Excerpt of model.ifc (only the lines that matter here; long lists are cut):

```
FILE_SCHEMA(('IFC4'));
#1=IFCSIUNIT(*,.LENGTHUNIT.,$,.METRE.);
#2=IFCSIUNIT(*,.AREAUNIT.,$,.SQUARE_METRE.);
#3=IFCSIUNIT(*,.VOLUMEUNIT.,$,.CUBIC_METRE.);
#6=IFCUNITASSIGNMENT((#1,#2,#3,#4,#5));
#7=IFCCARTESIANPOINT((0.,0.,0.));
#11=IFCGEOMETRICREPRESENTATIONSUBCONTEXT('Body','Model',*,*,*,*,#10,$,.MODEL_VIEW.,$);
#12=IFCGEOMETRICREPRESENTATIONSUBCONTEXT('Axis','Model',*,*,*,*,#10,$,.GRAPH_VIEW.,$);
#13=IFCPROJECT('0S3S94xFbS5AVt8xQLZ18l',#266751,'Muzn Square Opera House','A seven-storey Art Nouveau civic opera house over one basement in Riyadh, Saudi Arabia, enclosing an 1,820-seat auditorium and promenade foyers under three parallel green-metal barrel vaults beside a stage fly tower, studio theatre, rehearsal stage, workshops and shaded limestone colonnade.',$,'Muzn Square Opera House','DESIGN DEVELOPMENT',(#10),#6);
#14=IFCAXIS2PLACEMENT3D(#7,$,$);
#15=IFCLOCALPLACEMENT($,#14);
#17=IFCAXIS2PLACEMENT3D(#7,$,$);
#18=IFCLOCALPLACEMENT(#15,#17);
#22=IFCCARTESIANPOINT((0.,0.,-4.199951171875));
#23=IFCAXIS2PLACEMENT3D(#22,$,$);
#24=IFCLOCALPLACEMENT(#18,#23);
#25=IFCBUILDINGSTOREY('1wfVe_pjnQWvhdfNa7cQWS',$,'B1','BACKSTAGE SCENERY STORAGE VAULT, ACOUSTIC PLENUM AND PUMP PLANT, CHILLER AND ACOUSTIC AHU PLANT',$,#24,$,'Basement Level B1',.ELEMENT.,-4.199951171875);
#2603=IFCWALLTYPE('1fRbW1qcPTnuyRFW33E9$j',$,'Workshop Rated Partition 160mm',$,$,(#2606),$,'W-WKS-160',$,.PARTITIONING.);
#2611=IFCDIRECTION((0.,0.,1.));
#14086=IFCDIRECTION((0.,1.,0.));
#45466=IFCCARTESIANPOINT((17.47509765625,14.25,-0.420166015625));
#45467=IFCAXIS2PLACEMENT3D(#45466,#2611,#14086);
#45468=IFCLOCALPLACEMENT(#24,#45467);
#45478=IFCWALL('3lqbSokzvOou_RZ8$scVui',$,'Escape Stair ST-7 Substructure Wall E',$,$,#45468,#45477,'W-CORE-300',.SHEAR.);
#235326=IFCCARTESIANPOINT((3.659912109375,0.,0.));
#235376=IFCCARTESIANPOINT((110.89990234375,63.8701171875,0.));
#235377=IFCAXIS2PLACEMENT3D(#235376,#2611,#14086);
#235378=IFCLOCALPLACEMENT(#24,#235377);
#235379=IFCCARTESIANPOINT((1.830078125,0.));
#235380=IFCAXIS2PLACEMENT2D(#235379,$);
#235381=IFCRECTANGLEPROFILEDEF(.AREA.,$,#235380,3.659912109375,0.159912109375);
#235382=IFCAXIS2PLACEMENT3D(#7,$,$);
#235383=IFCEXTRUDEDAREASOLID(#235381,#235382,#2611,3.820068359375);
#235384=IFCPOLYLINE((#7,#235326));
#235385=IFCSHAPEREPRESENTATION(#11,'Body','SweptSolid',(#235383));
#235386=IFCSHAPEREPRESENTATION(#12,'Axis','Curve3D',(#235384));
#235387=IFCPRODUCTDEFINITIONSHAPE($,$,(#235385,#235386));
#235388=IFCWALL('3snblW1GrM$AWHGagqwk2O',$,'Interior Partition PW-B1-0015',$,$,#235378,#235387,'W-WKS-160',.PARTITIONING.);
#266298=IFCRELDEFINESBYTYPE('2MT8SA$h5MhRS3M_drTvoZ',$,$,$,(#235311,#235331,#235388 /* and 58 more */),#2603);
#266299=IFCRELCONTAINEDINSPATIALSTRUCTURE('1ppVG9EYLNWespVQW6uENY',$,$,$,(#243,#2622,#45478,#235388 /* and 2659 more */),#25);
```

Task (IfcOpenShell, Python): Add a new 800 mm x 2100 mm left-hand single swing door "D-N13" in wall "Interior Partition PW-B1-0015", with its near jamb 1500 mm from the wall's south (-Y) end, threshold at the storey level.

```python
import numpy as np
import ifcopenshell
import ifcopenshell.api.feature
import ifcopenshell.api.geometry
import ifcopenshell.api.root
import ifcopenshell.api.spatial
import ifcopenshell.geom
import ifcopenshell.util.element
import ifcopenshell.util.placement
import ifcopenshell.util.representation
import ifcopenshell.util.shape
import ifcopenshell.util.unit

model = ifcopenshell.open("model.ifc")
unit_scale = ifcopenshell.util.unit.calculate_unit_scale(model)
settings = ifcopenshell.geom.settings()


def volume(element):
    """Net volume in cubic metres, openings subtracted."""
    shape = ifcopenshell.geom.create_shape(settings, element)
    return ifcopenshell.util.shape.get_volume(shape.geometry)


wall = model.by_guid("3snblW1GrM$AWHGagqwk2O")
storey = ifcopenshell.util.element.get_container(wall, ifc_class="IfcBuildingStorey")
context = ifcopenshell.util.representation.get_context(model, "Model", "Body", "MODEL_VIEW")
before = volume(wall)

width, height, from_end, sill = 0.8, 2.1, 1.5, 0.0  # metres

# The wall runs along its own X axis, and the end named is its -X end.
wall_shape = ifcopenshell.geom.create_shape(settings, wall)
x, y, z = ifcopenshell.util.shape.get_vertices(wall_shape.geometry).T
start = x.min() + from_end
face, thickness = float(y.min()), float(y.max() - y.min())
wall_matrix = ifcopenshell.util.placement.get_local_placement(wall.ObjectPlacement)
level = ifcopenshell.util.placement.get_local_placement(storey.ObjectPlacement)[2, 3]


def in_wall(x, y):
    """Placement at x, y metres in the wall's axes, at sill height."""
    matrix = wall_matrix.copy()
    matrix[:, 3] = wall_matrix @ np.array([x / unit_scale, y / unit_scale, 0.0, 1.0])
    matrix[2, 3] = level + sill / unit_scale
    return matrix


# Opening: a box that overshoots both wall faces by 50 mm.
opening = ifcopenshell.api.root.create_entity(model, ifc_class="IfcOpeningElement", predefined_type="OPENING")
box = ifcopenshell.api.geometry.add_wall_representation(
    model, context=context, length=width, height=height, thickness=thickness + 0.1
)
ifcopenshell.api.geometry.assign_representation(model, product=opening, representation=box)
ifcopenshell.api.geometry.edit_object_placement(model, product=opening, matrix=in_wall(start, face - 0.05), is_si=False)
ifcopenshell.api.feature.add_feature(model, feature=opening, element=wall)

door = ifcopenshell.api.root.create_entity(model, ifc_class="IfcDoor", name="D-N13", predefined_type="DOOR")
door.OverallWidth, door.OverallHeight = width / unit_scale, height / unit_scale
door.OperationType = "SINGLE_SWING_LEFT"
body = ifcopenshell.api.geometry.add_door_representation(
    model,
    context=context,
    overall_width=door.OverallWidth,
    overall_height=door.OverallHeight,
    operation_type="SINGLE_SWING_LEFT",
    lining_properties={"LiningDepth": thickness / unit_scale, "ThresholdDepth": thickness / unit_scale},
)
ifcopenshell.api.geometry.assign_representation(model, product=door, representation=body)
ifcopenshell.api.spatial.assign_container(model, products=[door], relating_structure=storey)
ifcopenshell.api.feature.add_filling(model, opening=opening, element=door)

# The lining spans the wall, so the door starts at the wall face.
ifcopenshell.api.geometry.edit_object_placement(model, product=door, matrix=in_wall(start, face), is_si=False)

after = volume(wall)

print(f"wall volume {before:.3f} -> {after:.3f} m3")

model.write("model_edited.ifc")
```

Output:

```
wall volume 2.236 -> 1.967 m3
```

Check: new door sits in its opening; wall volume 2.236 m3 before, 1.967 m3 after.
